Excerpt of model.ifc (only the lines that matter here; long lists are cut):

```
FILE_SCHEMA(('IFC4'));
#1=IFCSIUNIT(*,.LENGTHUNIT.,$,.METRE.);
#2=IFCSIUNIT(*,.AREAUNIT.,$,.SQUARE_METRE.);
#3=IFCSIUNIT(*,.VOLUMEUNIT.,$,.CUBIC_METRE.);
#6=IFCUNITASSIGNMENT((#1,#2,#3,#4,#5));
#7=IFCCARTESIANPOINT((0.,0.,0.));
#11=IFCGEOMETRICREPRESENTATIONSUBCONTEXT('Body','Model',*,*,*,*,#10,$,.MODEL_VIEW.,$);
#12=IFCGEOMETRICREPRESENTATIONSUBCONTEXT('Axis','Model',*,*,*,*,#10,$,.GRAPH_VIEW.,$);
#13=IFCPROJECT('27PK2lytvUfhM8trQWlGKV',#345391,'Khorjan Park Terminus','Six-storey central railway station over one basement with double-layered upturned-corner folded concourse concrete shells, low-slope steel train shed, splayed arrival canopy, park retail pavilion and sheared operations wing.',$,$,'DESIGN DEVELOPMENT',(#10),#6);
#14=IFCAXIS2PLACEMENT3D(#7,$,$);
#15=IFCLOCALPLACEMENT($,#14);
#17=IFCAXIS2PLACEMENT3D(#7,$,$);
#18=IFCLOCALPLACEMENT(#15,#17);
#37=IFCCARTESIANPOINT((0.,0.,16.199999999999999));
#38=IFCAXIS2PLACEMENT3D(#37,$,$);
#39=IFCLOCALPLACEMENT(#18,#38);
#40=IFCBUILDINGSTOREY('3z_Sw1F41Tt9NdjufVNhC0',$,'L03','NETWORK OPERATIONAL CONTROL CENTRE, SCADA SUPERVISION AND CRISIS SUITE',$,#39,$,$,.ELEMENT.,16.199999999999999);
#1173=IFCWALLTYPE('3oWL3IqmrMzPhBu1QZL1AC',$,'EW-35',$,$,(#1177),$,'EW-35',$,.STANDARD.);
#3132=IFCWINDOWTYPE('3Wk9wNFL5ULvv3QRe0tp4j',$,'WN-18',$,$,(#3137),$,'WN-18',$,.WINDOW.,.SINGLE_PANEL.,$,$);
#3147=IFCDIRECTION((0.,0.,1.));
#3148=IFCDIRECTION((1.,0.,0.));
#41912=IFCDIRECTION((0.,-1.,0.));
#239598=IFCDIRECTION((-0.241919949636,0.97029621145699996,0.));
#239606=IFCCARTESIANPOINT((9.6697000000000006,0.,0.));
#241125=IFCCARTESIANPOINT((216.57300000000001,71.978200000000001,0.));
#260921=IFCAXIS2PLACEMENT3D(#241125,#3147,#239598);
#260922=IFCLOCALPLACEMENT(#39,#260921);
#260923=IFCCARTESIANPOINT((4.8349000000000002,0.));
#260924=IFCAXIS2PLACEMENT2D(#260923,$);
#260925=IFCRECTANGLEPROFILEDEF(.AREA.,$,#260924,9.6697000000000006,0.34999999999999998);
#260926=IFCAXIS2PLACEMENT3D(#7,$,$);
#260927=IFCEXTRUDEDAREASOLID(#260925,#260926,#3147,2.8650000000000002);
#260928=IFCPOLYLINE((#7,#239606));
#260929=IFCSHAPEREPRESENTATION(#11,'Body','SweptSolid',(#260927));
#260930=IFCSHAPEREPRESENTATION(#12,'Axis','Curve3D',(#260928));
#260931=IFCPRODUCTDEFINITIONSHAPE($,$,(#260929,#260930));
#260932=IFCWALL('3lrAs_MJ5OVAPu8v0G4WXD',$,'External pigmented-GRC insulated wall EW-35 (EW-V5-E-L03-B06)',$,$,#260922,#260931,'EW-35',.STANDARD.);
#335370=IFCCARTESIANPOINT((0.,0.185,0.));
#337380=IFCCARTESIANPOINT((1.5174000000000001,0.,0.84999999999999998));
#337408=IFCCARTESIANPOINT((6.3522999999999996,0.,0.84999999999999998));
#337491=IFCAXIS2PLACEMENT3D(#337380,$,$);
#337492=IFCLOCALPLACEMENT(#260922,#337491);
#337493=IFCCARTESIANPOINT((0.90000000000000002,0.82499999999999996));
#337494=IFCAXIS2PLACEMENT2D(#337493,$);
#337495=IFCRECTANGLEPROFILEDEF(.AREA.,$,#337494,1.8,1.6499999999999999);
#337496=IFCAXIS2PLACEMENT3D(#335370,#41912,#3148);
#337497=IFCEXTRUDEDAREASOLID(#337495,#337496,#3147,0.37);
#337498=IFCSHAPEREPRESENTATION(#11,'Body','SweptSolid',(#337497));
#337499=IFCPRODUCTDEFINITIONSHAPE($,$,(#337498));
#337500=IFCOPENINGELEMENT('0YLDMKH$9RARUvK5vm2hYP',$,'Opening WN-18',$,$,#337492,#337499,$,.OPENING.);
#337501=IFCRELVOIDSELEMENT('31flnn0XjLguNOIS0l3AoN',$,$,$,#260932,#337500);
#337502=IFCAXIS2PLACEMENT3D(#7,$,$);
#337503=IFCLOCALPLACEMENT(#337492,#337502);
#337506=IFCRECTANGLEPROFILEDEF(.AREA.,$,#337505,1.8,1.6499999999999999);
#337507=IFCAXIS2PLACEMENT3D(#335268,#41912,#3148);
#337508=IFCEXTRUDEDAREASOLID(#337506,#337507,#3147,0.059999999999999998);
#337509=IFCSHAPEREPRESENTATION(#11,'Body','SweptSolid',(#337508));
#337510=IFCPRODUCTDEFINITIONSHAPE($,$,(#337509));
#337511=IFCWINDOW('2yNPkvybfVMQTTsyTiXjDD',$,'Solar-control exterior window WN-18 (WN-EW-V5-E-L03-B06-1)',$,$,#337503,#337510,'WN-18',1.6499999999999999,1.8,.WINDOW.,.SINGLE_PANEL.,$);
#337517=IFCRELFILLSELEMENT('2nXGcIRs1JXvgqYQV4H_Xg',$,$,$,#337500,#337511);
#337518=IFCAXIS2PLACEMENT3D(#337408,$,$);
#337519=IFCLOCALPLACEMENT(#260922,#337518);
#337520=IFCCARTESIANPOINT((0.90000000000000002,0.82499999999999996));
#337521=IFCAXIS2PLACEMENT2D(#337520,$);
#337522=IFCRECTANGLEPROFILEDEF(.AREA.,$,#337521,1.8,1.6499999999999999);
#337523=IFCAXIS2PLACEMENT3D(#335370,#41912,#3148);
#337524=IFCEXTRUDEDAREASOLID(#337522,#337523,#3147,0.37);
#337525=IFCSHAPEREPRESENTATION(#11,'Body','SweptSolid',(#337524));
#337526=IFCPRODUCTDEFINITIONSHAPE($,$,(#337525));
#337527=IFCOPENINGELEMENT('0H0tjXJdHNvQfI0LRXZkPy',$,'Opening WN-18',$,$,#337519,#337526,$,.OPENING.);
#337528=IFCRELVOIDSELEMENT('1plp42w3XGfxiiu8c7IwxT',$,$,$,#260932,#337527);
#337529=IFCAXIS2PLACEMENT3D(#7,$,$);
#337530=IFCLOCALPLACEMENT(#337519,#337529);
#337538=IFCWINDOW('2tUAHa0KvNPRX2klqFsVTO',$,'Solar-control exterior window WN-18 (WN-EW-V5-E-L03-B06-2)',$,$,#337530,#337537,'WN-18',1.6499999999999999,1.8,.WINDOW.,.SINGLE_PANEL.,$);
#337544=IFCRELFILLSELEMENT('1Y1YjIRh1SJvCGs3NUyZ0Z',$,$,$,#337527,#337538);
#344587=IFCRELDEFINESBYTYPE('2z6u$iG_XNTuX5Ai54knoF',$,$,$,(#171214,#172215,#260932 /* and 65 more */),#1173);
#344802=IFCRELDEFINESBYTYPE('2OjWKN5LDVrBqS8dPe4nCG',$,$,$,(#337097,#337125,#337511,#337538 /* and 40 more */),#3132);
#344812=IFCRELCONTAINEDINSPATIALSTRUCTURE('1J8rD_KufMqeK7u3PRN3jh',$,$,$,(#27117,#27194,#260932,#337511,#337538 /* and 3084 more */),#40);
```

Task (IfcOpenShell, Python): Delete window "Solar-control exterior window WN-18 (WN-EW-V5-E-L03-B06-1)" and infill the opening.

```python
import ifcopenshell
import ifcopenshell.api.feature
import ifcopenshell.api.root
import ifcopenshell.geom
import ifcopenshell.util.shape

model = ifcopenshell.open("model.ifc")
settings = ifcopenshell.geom.settings()


def volume(element):
    """Net volume in cubic metres, openings subtracted."""
    shape = ifcopenshell.geom.create_shape(settings, element)
    return ifcopenshell.util.shape.get_volume(shape.geometry)


window = model.by_guid("2yNPkvybfVMQTTsyTiXjDD")
opening = window.FillsVoids[0].RelatingOpeningElement
wall = opening.VoidsElements[0].RelatingBuildingElement
before = volume(wall)

ifcopenshell.api.root.remove_product(model, product=window)
ifcopenshell.api.feature.remove_feature(model, feature=opening)

after = volume(wall)

print(f"wall volume {before:.3f} -> {after:.3f} m3")

model.write("model_updated.ifc")
```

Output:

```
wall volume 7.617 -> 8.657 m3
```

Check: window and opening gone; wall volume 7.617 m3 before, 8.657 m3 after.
